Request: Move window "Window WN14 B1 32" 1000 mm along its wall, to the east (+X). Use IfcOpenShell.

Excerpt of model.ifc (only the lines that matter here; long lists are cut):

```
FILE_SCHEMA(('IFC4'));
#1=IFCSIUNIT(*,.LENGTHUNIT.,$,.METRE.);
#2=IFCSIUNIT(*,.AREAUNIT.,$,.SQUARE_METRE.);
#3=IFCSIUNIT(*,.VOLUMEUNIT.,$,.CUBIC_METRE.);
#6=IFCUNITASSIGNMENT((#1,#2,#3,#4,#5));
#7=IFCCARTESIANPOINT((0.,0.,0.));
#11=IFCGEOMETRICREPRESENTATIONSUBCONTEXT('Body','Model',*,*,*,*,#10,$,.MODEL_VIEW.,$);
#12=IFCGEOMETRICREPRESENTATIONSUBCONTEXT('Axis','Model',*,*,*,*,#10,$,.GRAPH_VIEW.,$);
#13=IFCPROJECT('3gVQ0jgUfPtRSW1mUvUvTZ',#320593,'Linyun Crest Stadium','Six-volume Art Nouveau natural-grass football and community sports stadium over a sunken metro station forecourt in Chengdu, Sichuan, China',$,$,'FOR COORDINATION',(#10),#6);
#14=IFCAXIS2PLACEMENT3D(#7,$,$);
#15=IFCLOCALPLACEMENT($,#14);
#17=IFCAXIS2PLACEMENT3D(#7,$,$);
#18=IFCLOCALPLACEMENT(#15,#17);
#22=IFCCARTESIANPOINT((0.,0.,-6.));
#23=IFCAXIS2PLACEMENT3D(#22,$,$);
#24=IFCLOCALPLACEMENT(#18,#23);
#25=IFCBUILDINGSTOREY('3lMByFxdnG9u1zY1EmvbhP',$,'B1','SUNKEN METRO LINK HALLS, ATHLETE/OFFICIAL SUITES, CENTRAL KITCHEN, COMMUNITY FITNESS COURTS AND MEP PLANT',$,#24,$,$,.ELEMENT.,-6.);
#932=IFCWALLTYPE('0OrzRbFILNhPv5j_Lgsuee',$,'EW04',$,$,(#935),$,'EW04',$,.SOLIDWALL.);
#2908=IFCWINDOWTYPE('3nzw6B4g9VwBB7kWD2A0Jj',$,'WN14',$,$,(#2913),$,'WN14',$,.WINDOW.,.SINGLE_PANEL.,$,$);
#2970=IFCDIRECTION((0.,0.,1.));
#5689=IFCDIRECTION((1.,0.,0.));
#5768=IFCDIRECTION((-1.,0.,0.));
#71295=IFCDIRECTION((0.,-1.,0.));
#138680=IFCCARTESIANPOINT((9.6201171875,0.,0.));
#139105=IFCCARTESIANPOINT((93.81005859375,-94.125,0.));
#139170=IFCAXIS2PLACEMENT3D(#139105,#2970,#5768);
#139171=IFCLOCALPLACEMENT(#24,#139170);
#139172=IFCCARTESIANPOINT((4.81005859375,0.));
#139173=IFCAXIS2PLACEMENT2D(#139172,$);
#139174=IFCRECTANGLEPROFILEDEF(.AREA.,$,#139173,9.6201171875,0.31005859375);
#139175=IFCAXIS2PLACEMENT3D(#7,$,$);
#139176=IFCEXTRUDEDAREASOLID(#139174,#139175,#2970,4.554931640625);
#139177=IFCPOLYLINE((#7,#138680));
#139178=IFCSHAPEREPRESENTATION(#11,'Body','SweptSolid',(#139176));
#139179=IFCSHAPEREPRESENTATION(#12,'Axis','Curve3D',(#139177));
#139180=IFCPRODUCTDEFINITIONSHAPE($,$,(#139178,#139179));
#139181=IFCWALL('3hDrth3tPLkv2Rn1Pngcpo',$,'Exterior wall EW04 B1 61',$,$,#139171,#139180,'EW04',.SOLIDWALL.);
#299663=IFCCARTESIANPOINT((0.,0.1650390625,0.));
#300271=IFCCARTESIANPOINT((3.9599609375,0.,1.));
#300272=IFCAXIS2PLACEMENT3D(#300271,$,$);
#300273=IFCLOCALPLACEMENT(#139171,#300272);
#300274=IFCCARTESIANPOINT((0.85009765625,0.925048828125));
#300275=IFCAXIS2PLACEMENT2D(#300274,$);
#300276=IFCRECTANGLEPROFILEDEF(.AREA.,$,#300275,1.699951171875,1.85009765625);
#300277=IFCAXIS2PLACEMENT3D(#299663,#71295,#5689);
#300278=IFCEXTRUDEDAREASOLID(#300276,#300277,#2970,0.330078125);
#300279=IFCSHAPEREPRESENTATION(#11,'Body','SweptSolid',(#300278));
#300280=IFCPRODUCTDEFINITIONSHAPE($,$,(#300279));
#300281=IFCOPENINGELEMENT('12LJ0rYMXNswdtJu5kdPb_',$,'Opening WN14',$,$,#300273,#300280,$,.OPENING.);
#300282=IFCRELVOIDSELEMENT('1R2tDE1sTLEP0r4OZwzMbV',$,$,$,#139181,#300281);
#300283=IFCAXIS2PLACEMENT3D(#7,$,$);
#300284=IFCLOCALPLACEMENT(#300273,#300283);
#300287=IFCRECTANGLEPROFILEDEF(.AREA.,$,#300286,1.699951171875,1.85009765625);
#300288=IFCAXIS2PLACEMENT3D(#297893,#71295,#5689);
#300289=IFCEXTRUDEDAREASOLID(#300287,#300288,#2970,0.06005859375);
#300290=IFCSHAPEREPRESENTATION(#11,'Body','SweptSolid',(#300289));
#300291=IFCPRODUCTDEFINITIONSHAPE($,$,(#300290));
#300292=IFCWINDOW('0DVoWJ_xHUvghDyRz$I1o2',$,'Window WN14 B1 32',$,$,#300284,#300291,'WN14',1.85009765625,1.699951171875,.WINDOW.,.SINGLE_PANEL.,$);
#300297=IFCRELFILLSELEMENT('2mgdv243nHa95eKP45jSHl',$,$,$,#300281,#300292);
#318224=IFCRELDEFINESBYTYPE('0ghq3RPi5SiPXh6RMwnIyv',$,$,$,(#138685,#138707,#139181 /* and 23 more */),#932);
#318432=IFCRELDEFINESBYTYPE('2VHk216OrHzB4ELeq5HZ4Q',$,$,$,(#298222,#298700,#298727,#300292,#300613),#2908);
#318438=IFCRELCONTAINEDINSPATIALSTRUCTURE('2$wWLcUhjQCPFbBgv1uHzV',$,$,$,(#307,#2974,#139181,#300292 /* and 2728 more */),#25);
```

```python
import ifcopenshell
import ifcopenshell.api.geometry
import ifcopenshell.util.placement

model = ifcopenshell.open("model.ifc")

window = model.by_guid("0DVoWJ_xHUvghDyRz$I1o2")
opening = window.FillsVoids[0].RelatingOpeningElement
wall = opening.VoidsElements[0].RelatingBuildingElement

wall_matrix = ifcopenshell.util.placement.get_local_placement(wall.ObjectPlacement)
shift = wall_matrix[:3, 0] * -1.0
before = ifcopenshell.util.placement.get_local_placement(window.ObjectPlacement)[:3, 3].copy()

# The window is placed relative to its opening, so it follows when the opening moves.
matrix = ifcopenshell.util.placement.get_local_placement(opening.ObjectPlacement)
matrix[:3, 3] += shift
ifcopenshell.api.geometry.edit_object_placement(
    model, product=opening, matrix=matrix, is_si=False, should_transform_children=True
)

after = ifcopenshell.util.placement.get_local_placement(window.ObjectPlacement)[:3, 3]
print("window moved by", (after - before).round(3) + 0.0)

model.write("model_edited.ifc")
```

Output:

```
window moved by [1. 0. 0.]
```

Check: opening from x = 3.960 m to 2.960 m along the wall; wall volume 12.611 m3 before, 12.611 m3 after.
